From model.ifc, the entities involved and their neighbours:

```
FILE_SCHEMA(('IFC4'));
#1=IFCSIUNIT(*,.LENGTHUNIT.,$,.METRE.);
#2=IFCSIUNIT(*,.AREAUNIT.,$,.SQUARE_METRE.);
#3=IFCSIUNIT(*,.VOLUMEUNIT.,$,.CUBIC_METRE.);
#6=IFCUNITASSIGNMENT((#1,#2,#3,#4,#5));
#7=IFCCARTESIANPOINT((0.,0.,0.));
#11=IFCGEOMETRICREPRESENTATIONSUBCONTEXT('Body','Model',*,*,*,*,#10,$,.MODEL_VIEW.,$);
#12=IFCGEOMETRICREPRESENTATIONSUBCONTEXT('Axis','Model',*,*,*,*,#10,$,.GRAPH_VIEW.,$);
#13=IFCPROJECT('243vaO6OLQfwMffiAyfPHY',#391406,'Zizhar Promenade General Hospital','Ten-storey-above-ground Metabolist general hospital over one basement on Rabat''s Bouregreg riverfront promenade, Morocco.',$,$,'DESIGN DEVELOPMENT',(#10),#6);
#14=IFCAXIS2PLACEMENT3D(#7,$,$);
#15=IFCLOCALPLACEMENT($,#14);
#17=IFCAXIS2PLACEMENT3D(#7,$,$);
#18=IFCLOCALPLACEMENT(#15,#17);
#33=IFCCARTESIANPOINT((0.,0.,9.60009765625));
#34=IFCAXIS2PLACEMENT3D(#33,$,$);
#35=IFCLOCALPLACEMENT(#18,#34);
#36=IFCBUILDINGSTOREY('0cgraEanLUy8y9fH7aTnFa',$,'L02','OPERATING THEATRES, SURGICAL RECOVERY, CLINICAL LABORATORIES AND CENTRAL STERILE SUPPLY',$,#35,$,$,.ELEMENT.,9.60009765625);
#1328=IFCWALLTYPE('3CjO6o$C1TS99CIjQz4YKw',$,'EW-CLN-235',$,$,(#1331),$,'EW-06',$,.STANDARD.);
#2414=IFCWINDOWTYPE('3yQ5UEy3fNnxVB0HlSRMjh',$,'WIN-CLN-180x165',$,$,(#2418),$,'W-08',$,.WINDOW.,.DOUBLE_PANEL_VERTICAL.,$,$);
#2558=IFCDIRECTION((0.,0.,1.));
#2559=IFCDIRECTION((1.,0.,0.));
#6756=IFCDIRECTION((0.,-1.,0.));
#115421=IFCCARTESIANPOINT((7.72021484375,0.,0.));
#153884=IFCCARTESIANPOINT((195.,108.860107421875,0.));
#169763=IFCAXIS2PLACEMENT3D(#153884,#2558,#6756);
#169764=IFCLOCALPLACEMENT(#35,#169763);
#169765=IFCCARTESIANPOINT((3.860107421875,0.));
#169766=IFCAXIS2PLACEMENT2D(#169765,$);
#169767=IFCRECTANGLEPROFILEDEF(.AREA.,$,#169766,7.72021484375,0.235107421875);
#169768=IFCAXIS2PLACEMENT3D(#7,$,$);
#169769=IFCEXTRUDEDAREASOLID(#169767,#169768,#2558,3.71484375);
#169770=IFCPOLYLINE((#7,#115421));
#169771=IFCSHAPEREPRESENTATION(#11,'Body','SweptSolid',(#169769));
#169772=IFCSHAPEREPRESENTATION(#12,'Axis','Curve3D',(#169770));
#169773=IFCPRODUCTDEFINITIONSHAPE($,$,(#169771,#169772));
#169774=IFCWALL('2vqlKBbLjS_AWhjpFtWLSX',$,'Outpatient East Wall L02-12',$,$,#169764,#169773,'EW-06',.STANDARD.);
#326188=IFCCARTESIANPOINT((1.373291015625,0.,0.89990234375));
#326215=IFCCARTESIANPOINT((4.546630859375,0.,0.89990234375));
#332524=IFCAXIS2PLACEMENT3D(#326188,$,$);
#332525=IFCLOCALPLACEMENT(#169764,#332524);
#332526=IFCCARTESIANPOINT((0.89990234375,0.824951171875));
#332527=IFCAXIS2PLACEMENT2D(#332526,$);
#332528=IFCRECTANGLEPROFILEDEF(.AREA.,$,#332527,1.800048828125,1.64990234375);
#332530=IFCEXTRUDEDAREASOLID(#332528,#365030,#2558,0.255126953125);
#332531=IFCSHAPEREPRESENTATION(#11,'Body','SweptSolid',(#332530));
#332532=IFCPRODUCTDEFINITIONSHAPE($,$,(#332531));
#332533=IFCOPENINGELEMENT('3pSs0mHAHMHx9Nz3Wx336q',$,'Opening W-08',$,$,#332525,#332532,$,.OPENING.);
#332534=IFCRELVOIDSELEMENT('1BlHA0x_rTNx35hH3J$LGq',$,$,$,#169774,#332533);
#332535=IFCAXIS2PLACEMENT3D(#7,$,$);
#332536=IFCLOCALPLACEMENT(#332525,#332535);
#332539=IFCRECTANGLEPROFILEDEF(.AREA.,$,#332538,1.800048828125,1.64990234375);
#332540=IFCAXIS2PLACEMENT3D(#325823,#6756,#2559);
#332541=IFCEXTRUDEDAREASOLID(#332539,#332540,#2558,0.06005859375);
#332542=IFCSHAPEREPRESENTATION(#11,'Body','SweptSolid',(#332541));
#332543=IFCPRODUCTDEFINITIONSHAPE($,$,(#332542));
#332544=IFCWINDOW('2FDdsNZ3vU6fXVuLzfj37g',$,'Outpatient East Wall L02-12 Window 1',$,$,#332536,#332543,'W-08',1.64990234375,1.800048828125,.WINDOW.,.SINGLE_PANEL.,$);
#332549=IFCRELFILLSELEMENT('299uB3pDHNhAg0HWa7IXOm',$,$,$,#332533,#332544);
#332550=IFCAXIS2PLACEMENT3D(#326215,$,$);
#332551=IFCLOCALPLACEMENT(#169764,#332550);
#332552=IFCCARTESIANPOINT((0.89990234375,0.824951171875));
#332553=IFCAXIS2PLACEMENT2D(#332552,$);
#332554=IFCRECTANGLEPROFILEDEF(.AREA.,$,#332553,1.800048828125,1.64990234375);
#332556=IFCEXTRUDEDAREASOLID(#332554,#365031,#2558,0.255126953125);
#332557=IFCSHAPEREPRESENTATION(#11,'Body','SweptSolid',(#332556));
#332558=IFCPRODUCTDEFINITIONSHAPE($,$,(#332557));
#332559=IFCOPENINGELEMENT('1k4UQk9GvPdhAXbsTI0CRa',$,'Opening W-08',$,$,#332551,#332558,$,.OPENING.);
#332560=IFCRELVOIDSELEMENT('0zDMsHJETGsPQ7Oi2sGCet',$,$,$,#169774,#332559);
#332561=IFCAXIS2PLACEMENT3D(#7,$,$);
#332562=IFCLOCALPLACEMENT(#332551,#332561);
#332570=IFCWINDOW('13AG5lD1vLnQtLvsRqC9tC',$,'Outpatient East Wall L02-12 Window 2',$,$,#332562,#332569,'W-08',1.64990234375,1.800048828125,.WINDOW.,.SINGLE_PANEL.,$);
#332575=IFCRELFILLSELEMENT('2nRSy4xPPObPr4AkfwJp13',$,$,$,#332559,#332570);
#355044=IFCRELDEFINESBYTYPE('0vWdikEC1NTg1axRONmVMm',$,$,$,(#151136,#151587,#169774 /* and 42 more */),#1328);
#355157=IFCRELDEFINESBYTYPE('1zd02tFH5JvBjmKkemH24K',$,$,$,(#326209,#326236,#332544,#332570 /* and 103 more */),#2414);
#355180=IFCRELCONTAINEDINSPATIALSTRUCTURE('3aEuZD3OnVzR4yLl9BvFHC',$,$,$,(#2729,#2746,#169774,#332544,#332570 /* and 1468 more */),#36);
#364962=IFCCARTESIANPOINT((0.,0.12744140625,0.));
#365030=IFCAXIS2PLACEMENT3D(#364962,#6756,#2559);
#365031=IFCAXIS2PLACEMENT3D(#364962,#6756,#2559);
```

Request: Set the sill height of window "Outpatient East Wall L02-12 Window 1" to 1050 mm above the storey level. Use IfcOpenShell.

```python
import numpy as np
import ifcopenshell
import ifcopenshell.api.geometry
import ifcopenshell.geom
import ifcopenshell.util.element
import ifcopenshell.util.placement
import ifcopenshell.util.shape
import ifcopenshell.util.unit

model = ifcopenshell.open("model.ifc")
unit_scale = ifcopenshell.util.unit.calculate_unit_scale(model)

window = model.by_guid("2FDdsNZ3vU6fXVuLzfj37g")
opening = window.FillsVoids[0].RelatingOpeningElement
storey = ifcopenshell.util.element.get_container(window, ifc_class="IfcBuildingStorey")
level = ifcopenshell.util.placement.get_local_placement(storey.ObjectPlacement)[2, 3]

# The opening's origin need not be at the sill, so measure its lowest point.
shape = ifcopenshell.geom.create_shape(ifcopenshell.geom.settings(), opening)
bottom = ifcopenshell.util.shape.get_shape_bottom_elevation(shape, shape.geometry) / unit_scale
dz = level + 1.05 - bottom

shift = np.array([0.0, 0.0, dz])
# The window is placed relative to its opening, so it follows when the opening moves.
matrix = ifcopenshell.util.placement.get_local_placement(opening.ObjectPlacement)
matrix[:3, 3] += shift
ifcopenshell.api.geometry.edit_object_placement(
    model, product=opening, matrix=matrix, is_si=False, should_transform_children=True
)

print(f"moved by {dz * unit_scale:+.3f} m")

model.write("model_edited.ifc")
```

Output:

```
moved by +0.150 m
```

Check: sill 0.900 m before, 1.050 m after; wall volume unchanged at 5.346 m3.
